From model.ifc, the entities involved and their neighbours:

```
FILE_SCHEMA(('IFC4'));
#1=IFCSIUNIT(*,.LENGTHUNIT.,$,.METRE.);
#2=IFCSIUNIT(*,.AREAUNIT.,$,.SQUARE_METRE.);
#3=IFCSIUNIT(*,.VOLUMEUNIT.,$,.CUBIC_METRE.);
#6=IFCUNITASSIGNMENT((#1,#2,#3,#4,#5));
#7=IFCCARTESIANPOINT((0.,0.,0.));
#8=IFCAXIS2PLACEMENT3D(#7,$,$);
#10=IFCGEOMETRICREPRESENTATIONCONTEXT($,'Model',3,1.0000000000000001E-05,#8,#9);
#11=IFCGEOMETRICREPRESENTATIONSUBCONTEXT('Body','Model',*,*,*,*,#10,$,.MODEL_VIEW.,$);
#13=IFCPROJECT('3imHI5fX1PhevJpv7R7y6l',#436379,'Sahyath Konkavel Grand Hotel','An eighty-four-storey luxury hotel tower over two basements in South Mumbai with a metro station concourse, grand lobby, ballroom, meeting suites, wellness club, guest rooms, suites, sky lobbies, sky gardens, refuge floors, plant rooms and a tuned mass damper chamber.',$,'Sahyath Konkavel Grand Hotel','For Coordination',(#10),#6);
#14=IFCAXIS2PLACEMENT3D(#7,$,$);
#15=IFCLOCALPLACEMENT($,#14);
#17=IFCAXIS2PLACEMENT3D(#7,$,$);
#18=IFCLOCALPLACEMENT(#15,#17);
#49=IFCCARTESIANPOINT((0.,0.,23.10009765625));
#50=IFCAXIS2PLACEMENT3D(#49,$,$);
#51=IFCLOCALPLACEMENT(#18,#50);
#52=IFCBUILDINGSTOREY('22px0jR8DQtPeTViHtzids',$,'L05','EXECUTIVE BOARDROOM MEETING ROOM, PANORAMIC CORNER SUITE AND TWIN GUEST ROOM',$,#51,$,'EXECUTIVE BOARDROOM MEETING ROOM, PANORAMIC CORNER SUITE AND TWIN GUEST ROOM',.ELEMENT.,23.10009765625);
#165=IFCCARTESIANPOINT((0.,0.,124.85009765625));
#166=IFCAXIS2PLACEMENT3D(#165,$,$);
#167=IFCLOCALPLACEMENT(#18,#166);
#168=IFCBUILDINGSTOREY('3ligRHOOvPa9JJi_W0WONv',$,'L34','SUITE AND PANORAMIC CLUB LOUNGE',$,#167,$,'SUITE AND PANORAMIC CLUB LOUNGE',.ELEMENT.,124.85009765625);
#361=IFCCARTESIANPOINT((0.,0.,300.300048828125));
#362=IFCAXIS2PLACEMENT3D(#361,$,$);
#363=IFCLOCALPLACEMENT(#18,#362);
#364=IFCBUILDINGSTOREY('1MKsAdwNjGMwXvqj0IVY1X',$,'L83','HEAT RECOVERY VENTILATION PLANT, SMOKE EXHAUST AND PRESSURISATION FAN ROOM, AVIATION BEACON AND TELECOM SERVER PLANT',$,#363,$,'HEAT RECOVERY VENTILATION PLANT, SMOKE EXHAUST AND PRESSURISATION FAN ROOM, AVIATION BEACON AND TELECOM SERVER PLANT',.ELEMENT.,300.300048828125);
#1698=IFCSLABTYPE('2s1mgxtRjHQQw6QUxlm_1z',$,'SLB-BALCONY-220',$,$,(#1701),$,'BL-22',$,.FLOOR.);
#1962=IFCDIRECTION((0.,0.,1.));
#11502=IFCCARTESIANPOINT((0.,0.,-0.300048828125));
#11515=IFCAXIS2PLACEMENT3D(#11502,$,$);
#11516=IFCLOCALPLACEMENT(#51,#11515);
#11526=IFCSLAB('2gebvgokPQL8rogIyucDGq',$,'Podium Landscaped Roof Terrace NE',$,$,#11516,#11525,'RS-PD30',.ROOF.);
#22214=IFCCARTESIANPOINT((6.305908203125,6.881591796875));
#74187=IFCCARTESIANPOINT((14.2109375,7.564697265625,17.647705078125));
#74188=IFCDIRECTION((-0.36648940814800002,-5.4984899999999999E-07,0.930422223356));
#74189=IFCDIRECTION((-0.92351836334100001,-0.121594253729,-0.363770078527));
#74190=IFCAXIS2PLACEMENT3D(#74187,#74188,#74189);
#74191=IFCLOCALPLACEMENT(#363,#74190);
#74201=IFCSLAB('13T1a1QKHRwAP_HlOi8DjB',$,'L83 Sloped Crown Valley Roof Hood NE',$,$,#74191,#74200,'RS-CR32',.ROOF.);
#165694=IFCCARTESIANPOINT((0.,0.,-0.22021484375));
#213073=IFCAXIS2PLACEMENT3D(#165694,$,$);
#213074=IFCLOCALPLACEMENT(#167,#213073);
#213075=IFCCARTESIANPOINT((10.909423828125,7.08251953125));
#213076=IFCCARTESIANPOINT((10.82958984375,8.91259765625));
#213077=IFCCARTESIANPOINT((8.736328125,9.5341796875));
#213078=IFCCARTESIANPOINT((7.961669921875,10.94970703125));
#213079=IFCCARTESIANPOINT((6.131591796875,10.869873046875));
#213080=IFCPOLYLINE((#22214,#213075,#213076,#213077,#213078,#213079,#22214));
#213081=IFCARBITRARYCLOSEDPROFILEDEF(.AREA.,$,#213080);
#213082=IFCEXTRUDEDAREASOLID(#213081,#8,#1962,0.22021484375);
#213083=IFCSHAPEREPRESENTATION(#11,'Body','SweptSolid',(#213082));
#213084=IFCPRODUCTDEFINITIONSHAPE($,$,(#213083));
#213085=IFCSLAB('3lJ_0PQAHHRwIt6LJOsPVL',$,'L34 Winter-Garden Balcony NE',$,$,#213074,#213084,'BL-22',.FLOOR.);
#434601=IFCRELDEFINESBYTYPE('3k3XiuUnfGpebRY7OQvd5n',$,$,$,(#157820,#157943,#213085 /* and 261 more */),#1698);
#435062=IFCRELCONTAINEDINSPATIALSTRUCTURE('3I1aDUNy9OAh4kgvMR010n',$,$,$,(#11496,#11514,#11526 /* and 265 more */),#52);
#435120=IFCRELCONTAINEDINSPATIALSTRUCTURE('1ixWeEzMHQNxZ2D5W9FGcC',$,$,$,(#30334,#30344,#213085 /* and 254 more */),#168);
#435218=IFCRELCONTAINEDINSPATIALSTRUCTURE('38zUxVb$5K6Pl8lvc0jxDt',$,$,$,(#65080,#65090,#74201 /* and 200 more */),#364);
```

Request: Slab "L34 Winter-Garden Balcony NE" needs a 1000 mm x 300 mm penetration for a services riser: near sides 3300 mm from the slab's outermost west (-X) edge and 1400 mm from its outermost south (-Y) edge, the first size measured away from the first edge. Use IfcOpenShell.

```python
import numpy as np
import ifcopenshell
import ifcopenshell.api.feature
import ifcopenshell.api.geometry
import ifcopenshell.api.root
import ifcopenshell.geom
import ifcopenshell.util.placement
import ifcopenshell.util.representation
import ifcopenshell.util.shape
import ifcopenshell.util.unit

model = ifcopenshell.open("model.ifc")
unit_scale = ifcopenshell.util.unit.calculate_unit_scale(model)
settings = ifcopenshell.geom.settings()


def volume(element):
    """Net volume in cubic metres, openings subtracted."""
    shape = ifcopenshell.geom.create_shape(settings, element)
    return ifcopenshell.util.shape.get_volume(shape.geometry)


slab = model.by_guid("3lJ_0PQAHHRwIt6LJOsPVL")
before = volume(slab)

# Extent in the slab's own axes, in metres. The edges named are its -X and -Y sides.
slab_shape = ifcopenshell.geom.create_shape(settings, slab)
vertices = ifcopenshell.util.shape.get_vertices(slab_shape.geometry)
x_min, y_min, bottom = vertices.min(axis=0)
top = vertices[:, 2].max()

opening = ifcopenshell.api.root.create_entity(model, ifc_class="IfcOpeningElement", name="Services riser opening", predefined_type="OPENING")
context = ifcopenshell.util.representation.get_context(model, "Model", "Body", "MODEL_VIEW")
width, depth = 1, 0.3
outline = [(0.0, 0.0), (width, 0.0), (width, depth), (0.0, depth), (0.0, 0.0)]
# Overshoot both faces by 50 mm so the cut is clean.
shape = ifcopenshell.api.geometry.add_slab_representation(
    model, context=context, depth=top - bottom + 0.1, polyline=outline
)
ifcopenshell.api.geometry.assign_representation(model, product=opening, representation=shape)

matrix = ifcopenshell.util.placement.get_local_placement(slab.ObjectPlacement)
matrix[:, 3] = matrix @ np.append(np.array([x_min + 3.3, y_min + 1.4, bottom - 0.05]) / unit_scale, 1.0)
ifcopenshell.api.geometry.edit_object_placement(model, product=opening, matrix=matrix, is_si=False)
ifcopenshell.api.feature.add_feature(model, feature=opening, element=slab)

after = volume(slab)

print(f"slab volume {before:.3f} -> {after:.3f} m3")

model.write("model_updated.ifc")
```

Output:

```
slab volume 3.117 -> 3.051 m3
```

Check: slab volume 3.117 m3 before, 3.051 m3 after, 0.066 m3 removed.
